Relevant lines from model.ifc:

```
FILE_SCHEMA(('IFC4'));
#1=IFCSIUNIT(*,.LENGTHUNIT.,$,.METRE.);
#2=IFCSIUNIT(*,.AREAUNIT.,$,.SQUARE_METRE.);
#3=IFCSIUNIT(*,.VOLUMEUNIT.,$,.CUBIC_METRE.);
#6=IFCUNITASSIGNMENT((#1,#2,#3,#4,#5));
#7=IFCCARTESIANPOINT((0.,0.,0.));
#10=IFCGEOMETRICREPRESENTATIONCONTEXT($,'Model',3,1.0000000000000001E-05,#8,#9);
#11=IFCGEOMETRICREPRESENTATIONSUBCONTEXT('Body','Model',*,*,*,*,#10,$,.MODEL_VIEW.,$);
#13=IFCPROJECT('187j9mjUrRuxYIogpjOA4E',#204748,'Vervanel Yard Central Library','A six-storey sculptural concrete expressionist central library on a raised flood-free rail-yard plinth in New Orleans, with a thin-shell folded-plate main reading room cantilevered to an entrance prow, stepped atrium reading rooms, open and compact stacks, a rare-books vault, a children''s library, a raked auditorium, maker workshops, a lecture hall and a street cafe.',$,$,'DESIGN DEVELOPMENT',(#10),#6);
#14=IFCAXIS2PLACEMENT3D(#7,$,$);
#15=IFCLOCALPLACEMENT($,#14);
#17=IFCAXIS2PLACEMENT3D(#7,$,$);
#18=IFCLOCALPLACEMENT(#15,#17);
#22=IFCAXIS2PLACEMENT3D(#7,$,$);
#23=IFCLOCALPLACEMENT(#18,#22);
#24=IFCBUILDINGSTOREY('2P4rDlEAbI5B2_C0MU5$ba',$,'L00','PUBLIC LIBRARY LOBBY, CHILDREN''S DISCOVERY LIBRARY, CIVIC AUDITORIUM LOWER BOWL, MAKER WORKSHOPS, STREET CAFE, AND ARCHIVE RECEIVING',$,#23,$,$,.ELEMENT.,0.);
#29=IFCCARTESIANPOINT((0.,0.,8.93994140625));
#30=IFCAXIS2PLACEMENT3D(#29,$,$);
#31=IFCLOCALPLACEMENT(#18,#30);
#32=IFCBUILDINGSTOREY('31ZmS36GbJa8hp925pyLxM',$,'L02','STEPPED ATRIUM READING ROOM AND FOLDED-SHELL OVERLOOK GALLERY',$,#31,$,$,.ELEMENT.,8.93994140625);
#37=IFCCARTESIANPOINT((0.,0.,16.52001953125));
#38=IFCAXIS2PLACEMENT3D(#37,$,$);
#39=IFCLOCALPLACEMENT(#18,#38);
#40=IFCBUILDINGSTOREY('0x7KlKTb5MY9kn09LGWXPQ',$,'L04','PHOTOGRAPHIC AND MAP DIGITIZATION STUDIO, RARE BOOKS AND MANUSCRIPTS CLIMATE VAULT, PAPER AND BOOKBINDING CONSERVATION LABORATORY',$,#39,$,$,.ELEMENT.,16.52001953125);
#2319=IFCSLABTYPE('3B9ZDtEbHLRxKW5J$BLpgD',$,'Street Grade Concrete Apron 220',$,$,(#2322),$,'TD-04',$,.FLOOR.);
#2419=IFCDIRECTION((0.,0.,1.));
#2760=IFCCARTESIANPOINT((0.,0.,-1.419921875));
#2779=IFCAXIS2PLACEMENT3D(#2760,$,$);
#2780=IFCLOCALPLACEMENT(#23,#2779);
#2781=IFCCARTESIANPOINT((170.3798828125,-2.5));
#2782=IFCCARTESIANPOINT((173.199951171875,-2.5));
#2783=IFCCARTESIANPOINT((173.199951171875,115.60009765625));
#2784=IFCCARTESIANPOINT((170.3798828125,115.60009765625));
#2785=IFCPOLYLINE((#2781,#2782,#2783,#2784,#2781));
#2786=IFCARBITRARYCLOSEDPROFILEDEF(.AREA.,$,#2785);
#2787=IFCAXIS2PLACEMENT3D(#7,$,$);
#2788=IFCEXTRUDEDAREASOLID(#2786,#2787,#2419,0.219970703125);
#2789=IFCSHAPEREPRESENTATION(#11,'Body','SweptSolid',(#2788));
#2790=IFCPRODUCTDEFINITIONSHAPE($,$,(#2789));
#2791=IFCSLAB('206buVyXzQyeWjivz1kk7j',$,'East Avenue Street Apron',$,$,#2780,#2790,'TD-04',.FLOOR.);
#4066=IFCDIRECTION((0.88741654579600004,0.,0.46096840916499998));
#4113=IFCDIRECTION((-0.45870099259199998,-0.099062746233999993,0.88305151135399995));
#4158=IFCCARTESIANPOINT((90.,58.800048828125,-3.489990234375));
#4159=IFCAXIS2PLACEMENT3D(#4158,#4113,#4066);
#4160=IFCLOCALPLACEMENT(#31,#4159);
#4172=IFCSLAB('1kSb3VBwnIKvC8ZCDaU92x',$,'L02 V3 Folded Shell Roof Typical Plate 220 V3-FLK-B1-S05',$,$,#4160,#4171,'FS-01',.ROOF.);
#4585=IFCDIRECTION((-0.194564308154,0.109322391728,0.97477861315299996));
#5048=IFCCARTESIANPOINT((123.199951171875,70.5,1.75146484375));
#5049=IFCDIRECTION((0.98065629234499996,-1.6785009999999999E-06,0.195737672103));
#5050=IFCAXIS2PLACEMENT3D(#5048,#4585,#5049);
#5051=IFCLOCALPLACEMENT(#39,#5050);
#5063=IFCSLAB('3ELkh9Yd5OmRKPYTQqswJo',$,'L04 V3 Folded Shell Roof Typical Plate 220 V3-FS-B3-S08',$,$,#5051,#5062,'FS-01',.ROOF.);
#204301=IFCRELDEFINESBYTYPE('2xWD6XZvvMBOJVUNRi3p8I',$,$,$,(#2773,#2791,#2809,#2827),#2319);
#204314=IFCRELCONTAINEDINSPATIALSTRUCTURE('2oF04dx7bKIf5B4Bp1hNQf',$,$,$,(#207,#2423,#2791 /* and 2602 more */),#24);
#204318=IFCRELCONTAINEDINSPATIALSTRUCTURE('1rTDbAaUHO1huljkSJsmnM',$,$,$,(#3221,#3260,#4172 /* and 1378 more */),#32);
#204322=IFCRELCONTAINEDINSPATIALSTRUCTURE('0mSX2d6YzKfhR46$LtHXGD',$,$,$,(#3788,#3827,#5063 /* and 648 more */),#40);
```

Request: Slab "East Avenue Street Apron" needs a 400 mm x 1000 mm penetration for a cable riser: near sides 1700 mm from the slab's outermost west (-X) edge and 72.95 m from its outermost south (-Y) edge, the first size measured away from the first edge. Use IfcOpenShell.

```python
import numpy as np
import ifcopenshell
import ifcopenshell.api.feature
import ifcopenshell.api.geometry
import ifcopenshell.api.root
import ifcopenshell.geom
import ifcopenshell.util.placement
import ifcopenshell.util.representation
import ifcopenshell.util.shape
import ifcopenshell.util.unit

model = ifcopenshell.open("model.ifc")
unit_scale = ifcopenshell.util.unit.calculate_unit_scale(model)
settings = ifcopenshell.geom.settings()


def volume(element):
    """Net volume in cubic metres, openings subtracted."""
    shape = ifcopenshell.geom.create_shape(settings, element)
    return ifcopenshell.util.shape.get_volume(shape.geometry)


slab = model.by_id(2791)
before = volume(slab)

# Extent in the slab's own axes, in metres. The edges named are its -X and -Y sides.
slab_shape = ifcopenshell.geom.create_shape(settings, slab)
vertices = ifcopenshell.util.shape.get_vertices(slab_shape.geometry)
x_min, y_min, bottom = vertices.min(axis=0)
top = vertices[:, 2].max()

opening = ifcopenshell.api.root.create_entity(model, ifc_class="IfcOpeningElement", name="Cable riser opening", predefined_type="OPENING")
context = ifcopenshell.util.representation.get_context(model, "Model", "Body", "MODEL_VIEW")
width, depth = 0.4, 1
outline = [(0.0, 0.0), (width, 0.0), (width, depth), (0.0, depth), (0.0, 0.0)]
# Overshoot both faces by 50 mm so the cut is clean.
shape = ifcopenshell.api.geometry.add_slab_representation(
    model, context=context, depth=top - bottom + 0.1, polyline=outline
)
ifcopenshell.api.geometry.assign_representation(model, product=opening, representation=shape)

matrix = ifcopenshell.util.placement.get_local_placement(slab.ObjectPlacement)
matrix[:, 3] = matrix @ np.append(np.array([x_min + 1.7, y_min + 72.95, bottom - 0.05]) / unit_scale, 1.0)
ifcopenshell.api.geometry.edit_object_placement(model, product=opening, matrix=matrix, is_si=False)
ifcopenshell.api.feature.add_feature(model, feature=opening, element=slab)

after = volume(slab)

print(f"slab volume {before:.3f} -> {after:.3f} m3")

model.write("model_v2.ifc")
```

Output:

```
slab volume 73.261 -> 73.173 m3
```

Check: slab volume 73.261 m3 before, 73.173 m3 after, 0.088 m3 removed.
